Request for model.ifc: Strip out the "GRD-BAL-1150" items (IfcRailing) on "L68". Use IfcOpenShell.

First a look at what the model holds.

```python
import ifcopenshell
import ifcopenshell.util.element

model = ifcopenshell.open("model.ifc")
print(model.schema)
storey = next(s for s in model.by_type("IfcBuildingStorey") if s.Name == "L68")
railings = [e for e in ifcopenshell.util.element.get_decomposition(storey) if e.is_a("IfcRailing")]
seen = {}
for e in railings:
    element_type = ifcopenshell.util.element.get_type(e)
    name = element_type.Name if element_type not in (None, e) else None
    seen[name] = seen.get(name, 0) + 1
for name, count in sorted(seen.items(), key=str):
    print(count, "x", name)
```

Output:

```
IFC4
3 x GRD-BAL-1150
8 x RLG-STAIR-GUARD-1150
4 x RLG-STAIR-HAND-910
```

```python
import ifcopenshell
import ifcopenshell.api.root
import ifcopenshell.util.element

model = ifcopenshell.open("model.ifc")

storey = next(s for s in model.by_type("IfcBuildingStorey") if s.Name == "L68")
railings = [e for e in ifcopenshell.util.element.get_decomposition(storey) if e.is_a("IfcRailing")]
targets = [e for e in railings if (t := ifcopenshell.util.element.get_type(e)) not in (None, e) and t.Name == "GRD-BAL-1150"]

for e in targets:
    ifcopenshell.api.root.remove_product(model, product=e)
print(len(targets), "removed")

model.write("model_v2.ifc")
```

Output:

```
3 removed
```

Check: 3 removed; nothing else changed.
